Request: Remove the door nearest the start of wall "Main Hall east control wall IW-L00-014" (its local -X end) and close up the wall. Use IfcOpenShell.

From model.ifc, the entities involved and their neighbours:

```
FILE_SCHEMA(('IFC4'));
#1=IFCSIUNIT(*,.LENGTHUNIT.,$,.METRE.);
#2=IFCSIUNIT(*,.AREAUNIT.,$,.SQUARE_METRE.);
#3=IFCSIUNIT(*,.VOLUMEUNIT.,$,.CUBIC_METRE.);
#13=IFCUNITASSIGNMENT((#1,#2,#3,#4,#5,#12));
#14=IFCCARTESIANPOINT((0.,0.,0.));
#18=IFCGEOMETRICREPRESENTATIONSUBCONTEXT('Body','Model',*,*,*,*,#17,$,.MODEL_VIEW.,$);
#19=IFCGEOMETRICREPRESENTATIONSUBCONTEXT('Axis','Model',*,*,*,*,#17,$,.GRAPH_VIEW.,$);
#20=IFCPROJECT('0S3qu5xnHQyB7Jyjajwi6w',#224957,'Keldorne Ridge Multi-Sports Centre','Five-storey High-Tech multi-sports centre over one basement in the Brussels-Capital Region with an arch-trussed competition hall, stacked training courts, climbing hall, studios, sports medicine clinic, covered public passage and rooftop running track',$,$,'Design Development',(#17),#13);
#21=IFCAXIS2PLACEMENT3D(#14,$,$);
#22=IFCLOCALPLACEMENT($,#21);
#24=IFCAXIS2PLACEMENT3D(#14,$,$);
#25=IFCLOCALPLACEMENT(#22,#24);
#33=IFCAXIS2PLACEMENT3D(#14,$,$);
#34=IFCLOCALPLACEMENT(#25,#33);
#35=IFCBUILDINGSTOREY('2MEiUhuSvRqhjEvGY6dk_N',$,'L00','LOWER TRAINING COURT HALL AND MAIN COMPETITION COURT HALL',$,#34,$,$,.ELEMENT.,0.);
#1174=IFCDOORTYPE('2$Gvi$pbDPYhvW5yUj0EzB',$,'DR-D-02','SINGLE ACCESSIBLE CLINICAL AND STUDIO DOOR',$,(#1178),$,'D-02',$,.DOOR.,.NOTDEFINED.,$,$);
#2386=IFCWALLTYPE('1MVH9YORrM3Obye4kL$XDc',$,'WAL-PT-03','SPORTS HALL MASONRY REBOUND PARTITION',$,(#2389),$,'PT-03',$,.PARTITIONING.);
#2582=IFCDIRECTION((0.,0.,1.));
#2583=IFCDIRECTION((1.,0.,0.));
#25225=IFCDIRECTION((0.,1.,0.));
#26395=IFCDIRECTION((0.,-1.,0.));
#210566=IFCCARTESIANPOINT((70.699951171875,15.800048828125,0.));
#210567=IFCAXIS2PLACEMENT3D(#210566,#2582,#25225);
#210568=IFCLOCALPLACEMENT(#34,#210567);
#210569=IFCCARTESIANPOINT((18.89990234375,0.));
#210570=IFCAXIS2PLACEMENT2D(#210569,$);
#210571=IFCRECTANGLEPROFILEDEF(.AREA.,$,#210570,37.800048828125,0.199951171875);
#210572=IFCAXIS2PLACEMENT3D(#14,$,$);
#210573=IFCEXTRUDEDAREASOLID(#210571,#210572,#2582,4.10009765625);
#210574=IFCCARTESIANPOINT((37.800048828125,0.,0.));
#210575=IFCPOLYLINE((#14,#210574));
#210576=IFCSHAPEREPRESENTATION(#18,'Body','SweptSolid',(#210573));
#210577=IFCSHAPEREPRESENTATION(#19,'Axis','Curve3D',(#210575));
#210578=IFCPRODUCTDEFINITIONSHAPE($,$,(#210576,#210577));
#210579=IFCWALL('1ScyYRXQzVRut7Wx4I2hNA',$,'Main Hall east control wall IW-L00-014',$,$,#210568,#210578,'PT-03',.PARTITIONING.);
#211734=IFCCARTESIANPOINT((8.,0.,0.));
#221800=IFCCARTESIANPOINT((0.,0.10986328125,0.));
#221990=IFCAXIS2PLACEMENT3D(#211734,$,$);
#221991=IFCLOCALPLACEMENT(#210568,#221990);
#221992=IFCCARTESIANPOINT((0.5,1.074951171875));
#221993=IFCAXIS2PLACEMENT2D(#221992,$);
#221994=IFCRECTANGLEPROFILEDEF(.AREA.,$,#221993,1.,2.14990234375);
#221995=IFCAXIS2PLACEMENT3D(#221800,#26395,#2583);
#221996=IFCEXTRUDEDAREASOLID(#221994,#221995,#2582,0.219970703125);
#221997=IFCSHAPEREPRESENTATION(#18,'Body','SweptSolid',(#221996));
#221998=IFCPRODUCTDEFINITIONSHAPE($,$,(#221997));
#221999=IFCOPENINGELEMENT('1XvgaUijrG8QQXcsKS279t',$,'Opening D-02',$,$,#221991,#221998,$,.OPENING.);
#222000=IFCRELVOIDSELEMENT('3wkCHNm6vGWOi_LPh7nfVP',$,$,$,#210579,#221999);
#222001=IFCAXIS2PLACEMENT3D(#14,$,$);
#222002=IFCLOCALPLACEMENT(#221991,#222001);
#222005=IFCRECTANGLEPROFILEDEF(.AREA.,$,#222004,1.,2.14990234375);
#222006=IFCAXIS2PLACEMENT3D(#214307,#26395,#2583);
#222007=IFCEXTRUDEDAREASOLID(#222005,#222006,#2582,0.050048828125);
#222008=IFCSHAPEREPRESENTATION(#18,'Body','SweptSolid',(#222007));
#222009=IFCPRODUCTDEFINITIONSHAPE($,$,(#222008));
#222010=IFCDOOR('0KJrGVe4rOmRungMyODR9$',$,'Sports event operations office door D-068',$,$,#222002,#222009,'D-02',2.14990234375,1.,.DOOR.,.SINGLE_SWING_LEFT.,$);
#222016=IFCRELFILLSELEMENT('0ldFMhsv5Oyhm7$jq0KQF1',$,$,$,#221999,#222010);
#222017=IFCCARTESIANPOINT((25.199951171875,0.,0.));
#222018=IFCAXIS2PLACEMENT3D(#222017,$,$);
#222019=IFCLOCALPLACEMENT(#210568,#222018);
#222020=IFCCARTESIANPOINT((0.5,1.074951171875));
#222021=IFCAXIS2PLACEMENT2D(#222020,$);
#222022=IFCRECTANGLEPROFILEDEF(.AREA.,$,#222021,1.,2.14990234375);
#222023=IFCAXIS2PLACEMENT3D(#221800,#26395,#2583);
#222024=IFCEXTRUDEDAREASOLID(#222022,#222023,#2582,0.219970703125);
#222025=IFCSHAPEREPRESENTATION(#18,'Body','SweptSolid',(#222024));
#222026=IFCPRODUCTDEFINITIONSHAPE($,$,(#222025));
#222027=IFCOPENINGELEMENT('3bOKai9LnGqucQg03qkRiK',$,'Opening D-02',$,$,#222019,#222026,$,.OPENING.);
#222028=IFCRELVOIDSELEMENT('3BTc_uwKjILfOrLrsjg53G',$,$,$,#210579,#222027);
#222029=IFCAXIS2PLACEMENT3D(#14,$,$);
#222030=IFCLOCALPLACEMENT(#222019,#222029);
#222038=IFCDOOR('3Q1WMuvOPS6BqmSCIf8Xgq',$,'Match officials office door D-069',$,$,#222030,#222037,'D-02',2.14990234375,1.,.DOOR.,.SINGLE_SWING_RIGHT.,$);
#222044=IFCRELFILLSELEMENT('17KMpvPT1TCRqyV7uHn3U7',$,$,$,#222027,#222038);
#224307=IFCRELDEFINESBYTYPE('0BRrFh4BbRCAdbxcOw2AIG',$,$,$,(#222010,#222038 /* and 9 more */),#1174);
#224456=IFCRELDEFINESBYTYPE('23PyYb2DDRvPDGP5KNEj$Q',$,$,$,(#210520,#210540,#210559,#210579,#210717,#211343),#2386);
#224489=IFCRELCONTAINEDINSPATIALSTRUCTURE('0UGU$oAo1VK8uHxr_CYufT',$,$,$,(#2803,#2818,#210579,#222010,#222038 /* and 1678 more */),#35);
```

```python
import ifcopenshell
import ifcopenshell.api.feature
import ifcopenshell.api.root
import ifcopenshell.geom
import ifcopenshell.util.shape

model = ifcopenshell.open("model.ifc")
settings = ifcopenshell.geom.settings()


def volume(element):
    """Net volume in cubic metres, openings subtracted."""
    shape = ifcopenshell.geom.create_shape(settings, element)
    return ifcopenshell.util.shape.get_volume(shape.geometry)


door = model.by_guid("0KJrGVe4rOmRungMyODR9$")
opening = door.FillsVoids[0].RelatingOpeningElement
wall = opening.VoidsElements[0].RelatingBuildingElement
before = volume(wall)

ifcopenshell.api.root.remove_product(model, product=door)
ifcopenshell.api.feature.remove_feature(model, feature=opening)

after = volume(wall)

print(f"wall volume {before:.3f} -> {after:.3f} m3")

model.write("model_edited.ifc")
```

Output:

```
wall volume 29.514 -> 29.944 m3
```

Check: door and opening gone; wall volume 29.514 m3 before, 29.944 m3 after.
